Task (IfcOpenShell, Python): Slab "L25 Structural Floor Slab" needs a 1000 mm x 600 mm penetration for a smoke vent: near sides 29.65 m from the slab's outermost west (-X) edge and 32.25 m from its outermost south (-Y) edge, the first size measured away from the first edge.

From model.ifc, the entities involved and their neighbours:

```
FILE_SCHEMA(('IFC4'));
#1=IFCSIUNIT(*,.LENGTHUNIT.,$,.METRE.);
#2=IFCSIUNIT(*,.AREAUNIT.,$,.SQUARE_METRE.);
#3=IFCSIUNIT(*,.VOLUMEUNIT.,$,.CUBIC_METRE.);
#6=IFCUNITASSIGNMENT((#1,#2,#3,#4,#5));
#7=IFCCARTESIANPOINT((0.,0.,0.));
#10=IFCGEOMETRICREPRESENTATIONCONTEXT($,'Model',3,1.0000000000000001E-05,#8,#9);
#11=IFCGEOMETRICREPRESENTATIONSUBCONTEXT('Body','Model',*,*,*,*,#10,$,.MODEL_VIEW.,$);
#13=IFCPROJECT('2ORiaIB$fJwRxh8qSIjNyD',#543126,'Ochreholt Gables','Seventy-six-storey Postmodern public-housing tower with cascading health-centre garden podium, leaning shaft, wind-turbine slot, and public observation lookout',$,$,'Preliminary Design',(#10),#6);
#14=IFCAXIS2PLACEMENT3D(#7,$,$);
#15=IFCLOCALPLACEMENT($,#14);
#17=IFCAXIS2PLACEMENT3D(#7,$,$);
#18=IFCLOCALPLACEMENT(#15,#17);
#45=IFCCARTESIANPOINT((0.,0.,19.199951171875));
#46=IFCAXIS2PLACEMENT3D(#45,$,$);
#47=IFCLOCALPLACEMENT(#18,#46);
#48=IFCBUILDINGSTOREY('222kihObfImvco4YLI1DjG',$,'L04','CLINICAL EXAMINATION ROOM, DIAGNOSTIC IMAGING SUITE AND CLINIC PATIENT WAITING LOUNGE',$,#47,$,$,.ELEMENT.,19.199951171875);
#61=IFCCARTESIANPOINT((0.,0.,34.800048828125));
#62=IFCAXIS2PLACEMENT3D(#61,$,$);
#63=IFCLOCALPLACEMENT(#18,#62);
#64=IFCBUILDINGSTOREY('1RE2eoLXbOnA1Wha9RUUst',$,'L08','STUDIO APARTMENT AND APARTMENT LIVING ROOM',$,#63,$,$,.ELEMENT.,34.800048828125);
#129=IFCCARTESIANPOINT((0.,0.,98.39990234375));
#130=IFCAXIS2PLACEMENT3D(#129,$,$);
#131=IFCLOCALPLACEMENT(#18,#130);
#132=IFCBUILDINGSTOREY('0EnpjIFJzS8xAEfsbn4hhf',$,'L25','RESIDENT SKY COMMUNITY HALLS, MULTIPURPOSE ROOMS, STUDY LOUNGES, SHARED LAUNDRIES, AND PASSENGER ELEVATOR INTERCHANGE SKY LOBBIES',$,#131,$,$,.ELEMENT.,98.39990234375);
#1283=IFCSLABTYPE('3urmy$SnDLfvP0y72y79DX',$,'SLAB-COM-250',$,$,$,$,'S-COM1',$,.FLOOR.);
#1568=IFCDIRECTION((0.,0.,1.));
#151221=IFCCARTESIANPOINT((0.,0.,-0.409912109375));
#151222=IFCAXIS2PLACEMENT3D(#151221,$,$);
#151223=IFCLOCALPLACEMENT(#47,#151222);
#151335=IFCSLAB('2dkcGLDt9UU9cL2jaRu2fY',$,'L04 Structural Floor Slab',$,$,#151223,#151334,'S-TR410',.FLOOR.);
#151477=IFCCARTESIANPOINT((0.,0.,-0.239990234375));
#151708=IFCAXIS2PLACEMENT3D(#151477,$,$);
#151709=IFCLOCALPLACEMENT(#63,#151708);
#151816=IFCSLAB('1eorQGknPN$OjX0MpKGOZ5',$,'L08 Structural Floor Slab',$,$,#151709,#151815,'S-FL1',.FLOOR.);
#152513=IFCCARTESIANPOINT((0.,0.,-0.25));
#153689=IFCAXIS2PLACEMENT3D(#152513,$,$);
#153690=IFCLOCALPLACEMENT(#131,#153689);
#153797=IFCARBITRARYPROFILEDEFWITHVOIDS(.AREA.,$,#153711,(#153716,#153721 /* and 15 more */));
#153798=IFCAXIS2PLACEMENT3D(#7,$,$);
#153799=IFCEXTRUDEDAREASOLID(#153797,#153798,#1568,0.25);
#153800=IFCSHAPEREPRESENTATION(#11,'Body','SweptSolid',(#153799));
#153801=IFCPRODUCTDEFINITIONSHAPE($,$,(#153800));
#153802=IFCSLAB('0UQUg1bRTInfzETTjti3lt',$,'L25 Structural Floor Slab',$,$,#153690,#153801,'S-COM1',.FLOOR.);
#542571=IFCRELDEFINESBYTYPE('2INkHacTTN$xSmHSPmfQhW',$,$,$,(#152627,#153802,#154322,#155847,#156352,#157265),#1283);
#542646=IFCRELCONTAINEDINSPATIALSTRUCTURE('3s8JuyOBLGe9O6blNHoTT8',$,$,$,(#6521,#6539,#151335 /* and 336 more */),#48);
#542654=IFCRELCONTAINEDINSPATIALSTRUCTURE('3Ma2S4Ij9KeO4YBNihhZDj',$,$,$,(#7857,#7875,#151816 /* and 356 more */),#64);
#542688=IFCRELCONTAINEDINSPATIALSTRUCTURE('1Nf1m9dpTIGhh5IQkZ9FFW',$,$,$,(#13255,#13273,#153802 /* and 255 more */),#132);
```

```python
import numpy as np
import ifcopenshell
import ifcopenshell.api.feature
import ifcopenshell.api.geometry
import ifcopenshell.api.root
import ifcopenshell.geom
import ifcopenshell.util.placement
import ifcopenshell.util.representation
import ifcopenshell.util.shape
import ifcopenshell.util.unit

model = ifcopenshell.open("model.ifc")
unit_scale = ifcopenshell.util.unit.calculate_unit_scale(model)
settings = ifcopenshell.geom.settings()


def volume(element):
    """Net volume in cubic metres, openings subtracted."""
    shape = ifcopenshell.geom.create_shape(settings, element)
    return ifcopenshell.util.shape.get_volume(shape.geometry)


slab = model.by_guid("0UQUg1bRTInfzETTjti3lt")
before = volume(slab)

# Extent in the slab's own axes, in metres. The edges named are its -X and -Y sides.
slab_shape = ifcopenshell.geom.create_shape(settings, slab)
vertices = ifcopenshell.util.shape.get_vertices(slab_shape.geometry)
x_min, y_min, bottom = vertices.min(axis=0)
top = vertices[:, 2].max()

opening = ifcopenshell.api.root.create_entity(model, ifc_class="IfcOpeningElement", name="Smoke vent opening", predefined_type="OPENING")
context = ifcopenshell.util.representation.get_context(model, "Model", "Body", "MODEL_VIEW")
width, depth = 1, 0.6
outline = [(0.0, 0.0), (width, 0.0), (width, depth), (0.0, depth), (0.0, 0.0)]
# Overshoot both faces by 50 mm so the cut is clean.
shape = ifcopenshell.api.geometry.add_slab_representation(
    model, context=context, depth=top - bottom + 0.1, polyline=outline
)
ifcopenshell.api.geometry.assign_representation(model, product=opening, representation=shape)

matrix = ifcopenshell.util.placement.get_local_placement(slab.ObjectPlacement)
matrix[:, 3] = matrix @ np.append(np.array([x_min + 29.65, y_min + 32.25, bottom - 0.05]) / unit_scale, 1.0)
ifcopenshell.api.geometry.edit_object_placement(model, product=opening, matrix=matrix, is_si=False)
ifcopenshell.api.feature.add_feature(model, feature=opening, element=slab)

after = volume(slab)

print(f"slab volume {before:.3f} -> {after:.3f} m3")

model.write("model_v2.ifc")
```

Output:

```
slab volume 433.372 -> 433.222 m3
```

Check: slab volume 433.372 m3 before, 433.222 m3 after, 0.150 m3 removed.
